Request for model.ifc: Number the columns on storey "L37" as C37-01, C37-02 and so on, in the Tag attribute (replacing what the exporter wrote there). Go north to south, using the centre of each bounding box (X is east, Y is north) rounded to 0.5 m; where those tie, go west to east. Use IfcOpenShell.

First a look at what the model holds.

```python
import ifcopenshell
import ifcopenshell.util.element
import ifcopenshell.util.placement

model = ifcopenshell.open("model.ifc")
print(model.schema)
storey = next(s for s in model.by_type("IfcBuildingStorey") if s.Name == "L37")
columns = [e for e in ifcopenshell.util.element.get_decomposition(storey) if e.is_a("IfcColumn")]
for e in sorted(columns, key=lambda e: e.id()):
    origin = ifcopenshell.util.placement.get_local_placement(e.ObjectPlacement)[:3, 3]
    print(e.id(), e.Tag, e.Name, origin.round(2) + 0.0, sep=" | ")
```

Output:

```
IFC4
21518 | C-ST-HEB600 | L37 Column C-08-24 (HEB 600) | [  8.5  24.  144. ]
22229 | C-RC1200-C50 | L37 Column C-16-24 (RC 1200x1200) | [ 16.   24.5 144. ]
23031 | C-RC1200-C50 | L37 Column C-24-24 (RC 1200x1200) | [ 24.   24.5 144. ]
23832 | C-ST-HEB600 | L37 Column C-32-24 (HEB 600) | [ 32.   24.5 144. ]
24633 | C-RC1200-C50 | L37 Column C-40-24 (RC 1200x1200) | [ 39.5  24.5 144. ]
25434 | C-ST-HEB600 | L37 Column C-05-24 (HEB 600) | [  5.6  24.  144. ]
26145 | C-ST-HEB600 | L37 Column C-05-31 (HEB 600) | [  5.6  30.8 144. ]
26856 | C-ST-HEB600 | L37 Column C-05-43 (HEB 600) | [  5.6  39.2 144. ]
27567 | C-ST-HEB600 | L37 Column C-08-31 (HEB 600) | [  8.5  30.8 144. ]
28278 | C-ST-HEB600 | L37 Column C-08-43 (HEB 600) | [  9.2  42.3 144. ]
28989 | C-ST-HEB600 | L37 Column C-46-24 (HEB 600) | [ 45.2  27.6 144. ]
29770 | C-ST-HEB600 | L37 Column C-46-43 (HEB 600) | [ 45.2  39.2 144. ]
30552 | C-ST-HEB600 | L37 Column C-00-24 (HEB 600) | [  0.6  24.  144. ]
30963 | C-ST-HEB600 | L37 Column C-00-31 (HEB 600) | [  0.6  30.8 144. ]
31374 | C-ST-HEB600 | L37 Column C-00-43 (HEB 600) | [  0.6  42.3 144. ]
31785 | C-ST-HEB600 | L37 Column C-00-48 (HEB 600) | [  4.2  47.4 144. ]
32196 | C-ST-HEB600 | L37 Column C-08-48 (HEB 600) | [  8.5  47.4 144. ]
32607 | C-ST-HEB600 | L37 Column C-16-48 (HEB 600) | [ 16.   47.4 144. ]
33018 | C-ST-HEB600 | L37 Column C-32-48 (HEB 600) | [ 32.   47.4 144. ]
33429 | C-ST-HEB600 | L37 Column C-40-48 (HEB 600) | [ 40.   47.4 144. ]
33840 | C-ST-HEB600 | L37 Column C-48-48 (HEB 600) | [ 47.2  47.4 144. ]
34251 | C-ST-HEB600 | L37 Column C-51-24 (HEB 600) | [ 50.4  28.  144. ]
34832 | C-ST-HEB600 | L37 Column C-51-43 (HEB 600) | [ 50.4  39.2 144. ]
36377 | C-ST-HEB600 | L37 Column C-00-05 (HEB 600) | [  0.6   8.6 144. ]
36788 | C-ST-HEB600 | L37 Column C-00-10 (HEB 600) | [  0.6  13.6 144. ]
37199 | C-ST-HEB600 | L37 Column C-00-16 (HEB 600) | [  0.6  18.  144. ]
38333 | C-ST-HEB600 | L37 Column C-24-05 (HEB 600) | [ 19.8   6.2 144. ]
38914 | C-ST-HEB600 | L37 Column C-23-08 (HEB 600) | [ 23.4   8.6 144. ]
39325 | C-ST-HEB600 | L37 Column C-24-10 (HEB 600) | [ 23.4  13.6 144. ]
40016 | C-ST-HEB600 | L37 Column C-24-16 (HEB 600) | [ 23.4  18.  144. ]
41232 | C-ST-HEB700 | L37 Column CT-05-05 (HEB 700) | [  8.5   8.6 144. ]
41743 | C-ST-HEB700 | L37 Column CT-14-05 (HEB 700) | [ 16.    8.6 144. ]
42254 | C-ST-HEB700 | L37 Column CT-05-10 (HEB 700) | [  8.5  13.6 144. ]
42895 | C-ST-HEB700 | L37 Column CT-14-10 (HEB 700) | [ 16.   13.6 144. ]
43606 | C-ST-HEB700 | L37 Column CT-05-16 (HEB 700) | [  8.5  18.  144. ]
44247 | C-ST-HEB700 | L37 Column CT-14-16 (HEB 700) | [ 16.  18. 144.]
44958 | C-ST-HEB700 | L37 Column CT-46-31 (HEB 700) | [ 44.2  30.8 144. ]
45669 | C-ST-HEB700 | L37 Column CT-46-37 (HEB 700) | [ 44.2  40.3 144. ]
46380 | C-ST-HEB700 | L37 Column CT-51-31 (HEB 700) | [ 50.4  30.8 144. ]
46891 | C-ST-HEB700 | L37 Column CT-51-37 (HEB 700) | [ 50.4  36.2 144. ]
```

```python
import ifcopenshell
import ifcopenshell.geom
import ifcopenshell.util.element
import ifcopenshell.util.shape

model = ifcopenshell.open("model.ifc")
settings = ifcopenshell.geom.settings()
settings.set("use-world-coords", True)


def centre(element):
    shape = ifcopenshell.geom.create_shape(settings, element)
    return ifcopenshell.util.shape.get_bbox_centroid(shape.geometry)


storey = next(s for s in model.by_type("IfcBuildingStorey") if s.Name == "L37")
columns = [e for e in ifcopenshell.util.element.get_decomposition(storey) if e.is_a("IfcColumn")]

# Insertion points can sit at a corner or the storey origin, so sort by the geometry (in metres).
centres = {e: centre(e) for e in columns}
columns.sort(key=lambda e: (-round(centres[e][1] / 0.5), centres[e][0]))

for i, e in enumerate(columns, start=1):
    number = f"C37-{i:02d}"
    e.Tag = number
    print(e.id(), number)

model.write("model_updated.ifc")
```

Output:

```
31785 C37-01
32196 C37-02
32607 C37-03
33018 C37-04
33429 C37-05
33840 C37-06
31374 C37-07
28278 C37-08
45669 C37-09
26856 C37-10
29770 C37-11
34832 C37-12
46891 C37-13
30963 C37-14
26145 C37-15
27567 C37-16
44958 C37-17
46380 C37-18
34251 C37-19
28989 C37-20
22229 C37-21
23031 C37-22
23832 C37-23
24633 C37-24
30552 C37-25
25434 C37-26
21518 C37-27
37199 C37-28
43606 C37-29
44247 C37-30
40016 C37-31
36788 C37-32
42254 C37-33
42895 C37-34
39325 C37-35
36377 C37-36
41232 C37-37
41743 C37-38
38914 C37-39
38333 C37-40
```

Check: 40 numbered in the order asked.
